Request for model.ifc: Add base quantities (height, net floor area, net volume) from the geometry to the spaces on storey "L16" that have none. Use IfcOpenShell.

First a look at what the model holds.

```python
import ifcopenshell
import ifcopenshell.util.element
import ifcopenshell.util.unit

model = ifcopenshell.open("model.ifc")
print(model.schema)
for unit_type in ("LENGTHUNIT", "AREAUNIT", "VOLUMEUNIT"):
    print(unit_type, ifcopenshell.util.unit.calculate_unit_scale(model, unit_type))
storey = next(s for s in model.by_type("IfcBuildingStorey") if s.Name == "L16")
spaces = [e for e in ifcopenshell.util.element.get_decomposition(storey) if e.is_a("IfcSpace")]
for e in sorted(spaces, key=lambda e: e.id()):
    print(e.id(), e.is_a(), e.Name, list(ifcopenshell.util.element.get_psets(e, qtos_only=True)), sep=" | ")
```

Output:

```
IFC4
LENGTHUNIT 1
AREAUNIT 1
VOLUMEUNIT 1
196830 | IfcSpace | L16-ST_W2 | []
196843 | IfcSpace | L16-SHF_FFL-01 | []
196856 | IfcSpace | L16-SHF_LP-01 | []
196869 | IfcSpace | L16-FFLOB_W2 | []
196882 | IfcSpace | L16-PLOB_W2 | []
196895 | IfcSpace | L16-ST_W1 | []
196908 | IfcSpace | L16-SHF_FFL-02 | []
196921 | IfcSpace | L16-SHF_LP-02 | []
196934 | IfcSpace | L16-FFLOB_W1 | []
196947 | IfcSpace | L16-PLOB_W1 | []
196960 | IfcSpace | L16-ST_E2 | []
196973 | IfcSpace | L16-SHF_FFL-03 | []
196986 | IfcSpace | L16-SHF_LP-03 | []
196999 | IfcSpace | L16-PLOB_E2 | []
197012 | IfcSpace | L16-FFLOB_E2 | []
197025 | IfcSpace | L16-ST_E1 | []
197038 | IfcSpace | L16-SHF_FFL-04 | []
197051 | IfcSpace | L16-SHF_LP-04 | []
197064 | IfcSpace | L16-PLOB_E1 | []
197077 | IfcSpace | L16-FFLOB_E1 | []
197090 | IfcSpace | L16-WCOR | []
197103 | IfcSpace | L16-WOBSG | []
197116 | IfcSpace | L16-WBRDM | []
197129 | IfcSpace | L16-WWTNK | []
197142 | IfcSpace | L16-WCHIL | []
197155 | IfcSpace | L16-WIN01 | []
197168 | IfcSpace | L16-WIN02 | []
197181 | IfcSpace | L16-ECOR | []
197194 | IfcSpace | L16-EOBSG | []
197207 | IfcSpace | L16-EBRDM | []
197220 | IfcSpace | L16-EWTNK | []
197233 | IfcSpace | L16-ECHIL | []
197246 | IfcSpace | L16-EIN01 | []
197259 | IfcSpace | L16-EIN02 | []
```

```python
import ifcopenshell
import ifcopenshell.api.pset
import ifcopenshell.geom
import ifcopenshell.util.element
import ifcopenshell.util.shape
import ifcopenshell.util.unit

model = ifcopenshell.open("model.ifc")
unit_scale = ifcopenshell.util.unit.calculate_unit_scale(model)
area_scale = ifcopenshell.util.unit.calculate_unit_scale(model, "AREAUNIT")
volume_scale = ifcopenshell.util.unit.calculate_unit_scale(model, "VOLUMEUNIT")
settings = ifcopenshell.geom.settings()

storey = next(s for s in model.by_type("IfcBuildingStorey") if s.Name == "L16")
spaces = [e for e in ifcopenshell.util.element.get_decomposition(storey) if e.is_a("IfcSpace")]

for e in sorted(spaces, key=lambda e: e.id()):
    if ifcopenshell.util.element.get_psets(e, qtos_only=True, should_inherit=False):
        continue
    # Geometry comes back in metres, in the element's own axes.
    shape = ifcopenshell.geom.create_shape(settings, e)
    values = {
        "Height": ifcopenshell.util.shape.get_z(shape.geometry) / unit_scale,
        "NetFloorArea": ifcopenshell.util.shape.get_footprint_area(shape.geometry) / area_scale,
        "NetVolume": ifcopenshell.util.shape.get_volume(shape.geometry) / volume_scale,
    }
    qto = ifcopenshell.api.pset.add_qto(model, product=e, name="Qto_SpaceBaseQuantities")
    ifcopenshell.api.pset.edit_qto(model, qto=qto, properties=values)
    print(e.id(), {k: round(v, 3) for k, v in values.items()})

model.write("model_updated.ifc")
```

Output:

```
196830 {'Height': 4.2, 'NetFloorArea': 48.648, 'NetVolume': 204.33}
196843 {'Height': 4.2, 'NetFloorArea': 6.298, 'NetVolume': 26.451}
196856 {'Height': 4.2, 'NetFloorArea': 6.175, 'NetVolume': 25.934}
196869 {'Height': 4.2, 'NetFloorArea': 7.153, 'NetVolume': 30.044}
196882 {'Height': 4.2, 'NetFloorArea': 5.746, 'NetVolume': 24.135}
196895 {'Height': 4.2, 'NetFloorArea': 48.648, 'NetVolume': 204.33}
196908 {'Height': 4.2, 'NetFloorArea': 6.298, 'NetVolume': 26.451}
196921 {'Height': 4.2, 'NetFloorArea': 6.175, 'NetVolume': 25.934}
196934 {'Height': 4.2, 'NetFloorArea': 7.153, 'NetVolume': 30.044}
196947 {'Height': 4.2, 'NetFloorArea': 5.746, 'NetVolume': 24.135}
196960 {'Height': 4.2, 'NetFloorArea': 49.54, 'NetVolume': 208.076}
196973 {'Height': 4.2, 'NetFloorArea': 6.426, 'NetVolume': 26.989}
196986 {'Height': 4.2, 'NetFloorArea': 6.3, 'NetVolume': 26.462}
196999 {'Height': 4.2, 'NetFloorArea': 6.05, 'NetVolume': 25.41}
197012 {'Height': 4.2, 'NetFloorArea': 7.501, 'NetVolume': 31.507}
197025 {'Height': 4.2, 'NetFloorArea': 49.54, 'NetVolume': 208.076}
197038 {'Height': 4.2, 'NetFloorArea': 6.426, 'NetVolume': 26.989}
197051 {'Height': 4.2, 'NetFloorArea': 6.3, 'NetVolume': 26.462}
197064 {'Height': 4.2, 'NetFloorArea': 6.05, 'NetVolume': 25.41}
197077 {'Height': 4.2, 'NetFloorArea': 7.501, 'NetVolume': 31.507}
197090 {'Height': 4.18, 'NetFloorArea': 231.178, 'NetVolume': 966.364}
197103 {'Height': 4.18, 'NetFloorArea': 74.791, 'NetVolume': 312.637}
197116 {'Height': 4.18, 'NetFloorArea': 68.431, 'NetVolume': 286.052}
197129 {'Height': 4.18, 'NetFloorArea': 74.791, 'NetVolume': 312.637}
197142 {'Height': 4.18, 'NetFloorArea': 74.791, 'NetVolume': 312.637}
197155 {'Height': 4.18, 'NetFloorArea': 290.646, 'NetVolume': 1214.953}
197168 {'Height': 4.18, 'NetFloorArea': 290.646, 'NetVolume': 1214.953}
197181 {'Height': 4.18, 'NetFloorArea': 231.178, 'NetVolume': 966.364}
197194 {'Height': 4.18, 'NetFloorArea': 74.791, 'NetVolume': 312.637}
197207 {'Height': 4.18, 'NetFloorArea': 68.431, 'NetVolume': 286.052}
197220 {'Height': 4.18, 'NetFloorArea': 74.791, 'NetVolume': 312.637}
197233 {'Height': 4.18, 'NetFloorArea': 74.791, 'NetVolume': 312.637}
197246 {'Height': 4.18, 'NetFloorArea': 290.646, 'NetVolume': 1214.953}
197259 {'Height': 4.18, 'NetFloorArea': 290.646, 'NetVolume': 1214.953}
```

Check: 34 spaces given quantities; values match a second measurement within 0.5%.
